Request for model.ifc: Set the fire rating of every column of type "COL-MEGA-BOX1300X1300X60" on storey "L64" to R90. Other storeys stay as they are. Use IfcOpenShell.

First a look at what the model holds.

```python
import ifcopenshell
import ifcopenshell.util.element

model = ifcopenshell.open("model.ifc")
print(model.schema)
storey = next(s for s in model.by_type("IfcBuildingStorey") if s.Name == "L64")
columns = [e for e in ifcopenshell.util.element.get_decomposition(storey) if e.is_a("IfcColumn")]
seen = {}
for e in columns:
    element_type = ifcopenshell.util.element.get_type(e)
    key = (element_type.Name if element_type != e and element_type else None, ifcopenshell.util.element.get_pset(e, "Pset_ColumnCommon", "FireRating"))
    seen[key] = seen.get(key, 0) + 1
for (name, value), count in sorted(seen.items(), key=str):
    print(count, "x", name, "|", value)
```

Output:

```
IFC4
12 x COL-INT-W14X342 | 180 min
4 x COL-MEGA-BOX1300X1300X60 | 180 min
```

```python
import ifcopenshell
import ifcopenshell.api.pset
import ifcopenshell.util.element

model = ifcopenshell.open("model.ifc")

storey = next(s for s in model.by_type("IfcBuildingStorey") if s.Name == "L64")
columns = [e for e in ifcopenshell.util.element.get_decomposition(storey) if e.is_a("IfcColumn")]

count = 0
for e in columns:
    element_type = ifcopenshell.util.element.get_type(e)
    if element_type in (None, e) or element_type.Name != "COL-MEGA-BOX1300X1300X60":
        continue
    # add_pset returns the element's existing set when there is one.
    pset = ifcopenshell.api.pset.add_pset(model, product=e, name="Pset_ColumnCommon")
    ifcopenshell.api.pset.edit_pset(model, pset=pset, properties={"FireRating": "R90"})
    count += 1

print(count, "columns updated")

model.write("model_rev.ifc")
```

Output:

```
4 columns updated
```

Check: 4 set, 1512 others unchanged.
